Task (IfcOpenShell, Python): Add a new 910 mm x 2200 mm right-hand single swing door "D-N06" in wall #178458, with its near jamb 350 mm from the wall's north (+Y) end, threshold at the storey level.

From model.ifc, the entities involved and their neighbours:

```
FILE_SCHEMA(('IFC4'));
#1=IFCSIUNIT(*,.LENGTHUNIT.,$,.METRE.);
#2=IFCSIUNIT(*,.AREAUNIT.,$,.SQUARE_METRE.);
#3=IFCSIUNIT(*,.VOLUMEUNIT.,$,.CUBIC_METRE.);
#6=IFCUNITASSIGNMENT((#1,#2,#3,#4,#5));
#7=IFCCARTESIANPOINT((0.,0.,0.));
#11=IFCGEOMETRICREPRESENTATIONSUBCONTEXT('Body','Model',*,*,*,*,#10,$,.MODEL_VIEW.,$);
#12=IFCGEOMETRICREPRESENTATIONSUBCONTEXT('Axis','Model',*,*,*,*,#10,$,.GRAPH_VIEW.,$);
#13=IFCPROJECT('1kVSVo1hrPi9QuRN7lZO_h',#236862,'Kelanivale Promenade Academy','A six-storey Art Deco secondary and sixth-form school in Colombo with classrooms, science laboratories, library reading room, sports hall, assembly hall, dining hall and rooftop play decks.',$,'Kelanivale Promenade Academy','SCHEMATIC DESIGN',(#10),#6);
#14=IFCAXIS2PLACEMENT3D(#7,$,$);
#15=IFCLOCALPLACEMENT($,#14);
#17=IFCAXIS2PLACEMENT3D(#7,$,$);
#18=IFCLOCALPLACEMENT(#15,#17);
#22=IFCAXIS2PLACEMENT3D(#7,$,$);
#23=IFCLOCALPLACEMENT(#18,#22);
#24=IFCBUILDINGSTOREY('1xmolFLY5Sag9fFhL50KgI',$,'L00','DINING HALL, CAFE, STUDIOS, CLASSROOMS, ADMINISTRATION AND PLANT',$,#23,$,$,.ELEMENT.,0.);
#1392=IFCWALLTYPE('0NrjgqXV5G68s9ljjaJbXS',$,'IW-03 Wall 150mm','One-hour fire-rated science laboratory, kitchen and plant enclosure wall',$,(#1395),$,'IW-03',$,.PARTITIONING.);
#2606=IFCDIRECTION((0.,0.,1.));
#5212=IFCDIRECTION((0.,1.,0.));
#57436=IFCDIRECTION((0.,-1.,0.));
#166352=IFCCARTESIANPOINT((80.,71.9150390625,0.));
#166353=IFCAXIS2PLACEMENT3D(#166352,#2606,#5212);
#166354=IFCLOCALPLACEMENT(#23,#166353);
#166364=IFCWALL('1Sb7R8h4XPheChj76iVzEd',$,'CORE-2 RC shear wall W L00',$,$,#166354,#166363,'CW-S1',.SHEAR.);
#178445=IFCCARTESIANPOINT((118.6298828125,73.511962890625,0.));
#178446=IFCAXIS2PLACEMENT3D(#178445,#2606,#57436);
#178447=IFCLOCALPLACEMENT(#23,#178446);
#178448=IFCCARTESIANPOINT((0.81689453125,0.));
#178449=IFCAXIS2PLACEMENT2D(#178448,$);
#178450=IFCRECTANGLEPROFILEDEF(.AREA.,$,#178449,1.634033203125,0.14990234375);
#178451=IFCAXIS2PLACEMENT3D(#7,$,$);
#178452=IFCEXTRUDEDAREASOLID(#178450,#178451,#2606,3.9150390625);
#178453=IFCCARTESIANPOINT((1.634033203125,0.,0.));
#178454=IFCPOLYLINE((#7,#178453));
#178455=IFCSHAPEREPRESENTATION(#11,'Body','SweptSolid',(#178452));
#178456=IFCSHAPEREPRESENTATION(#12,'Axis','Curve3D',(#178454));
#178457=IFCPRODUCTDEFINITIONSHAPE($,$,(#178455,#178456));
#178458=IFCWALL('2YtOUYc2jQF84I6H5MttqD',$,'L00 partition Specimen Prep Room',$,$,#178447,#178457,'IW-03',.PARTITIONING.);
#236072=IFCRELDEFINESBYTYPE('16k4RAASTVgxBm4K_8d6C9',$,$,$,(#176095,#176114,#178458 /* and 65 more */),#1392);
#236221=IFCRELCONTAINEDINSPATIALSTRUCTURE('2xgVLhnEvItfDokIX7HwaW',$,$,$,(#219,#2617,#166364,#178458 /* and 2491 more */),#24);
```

```python
import numpy as np
import ifcopenshell
import ifcopenshell.api.feature
import ifcopenshell.api.geometry
import ifcopenshell.api.root
import ifcopenshell.api.spatial
import ifcopenshell.geom
import ifcopenshell.util.element
import ifcopenshell.util.placement
import ifcopenshell.util.representation
import ifcopenshell.util.shape
import ifcopenshell.util.unit

model = ifcopenshell.open("model.ifc")
unit_scale = ifcopenshell.util.unit.calculate_unit_scale(model)
settings = ifcopenshell.geom.settings()


def volume(element):
    """Net volume in cubic metres, openings subtracted."""
    shape = ifcopenshell.geom.create_shape(settings, element)
    return ifcopenshell.util.shape.get_volume(shape.geometry)


wall = model.by_guid("2YtOUYc2jQF84I6H5MttqD")
storey = ifcopenshell.util.element.get_container(wall, ifc_class="IfcBuildingStorey")
context = ifcopenshell.util.representation.get_context(model, "Model", "Body", "MODEL_VIEW")
before = volume(wall)

width, height, from_end, sill = 0.91, 2.2, 0.35, 0.0  # metres

# The wall runs along its own X axis, and the end named is its -X end.
wall_shape = ifcopenshell.geom.create_shape(settings, wall)
x, y, z = ifcopenshell.util.shape.get_vertices(wall_shape.geometry).T
start = x.min() + from_end
face, thickness = float(y.min()), float(y.max() - y.min())
wall_matrix = ifcopenshell.util.placement.get_local_placement(wall.ObjectPlacement)
level = ifcopenshell.util.placement.get_local_placement(storey.ObjectPlacement)[2, 3]


def in_wall(x, y):
    """Placement at x, y metres in the wall's axes, at sill height."""
    matrix = wall_matrix.copy()
    matrix[:, 3] = wall_matrix @ np.array([x / unit_scale, y / unit_scale, 0.0, 1.0])
    matrix[2, 3] = level + sill / unit_scale
    return matrix


# Opening: a box that overshoots both wall faces by 50 mm.
opening = ifcopenshell.api.root.create_entity(model, ifc_class="IfcOpeningElement", predefined_type="OPENING")
box = ifcopenshell.api.geometry.add_wall_representation(
    model, context=context, length=width, height=height, thickness=thickness + 0.1
)
ifcopenshell.api.geometry.assign_representation(model, product=opening, representation=box)
ifcopenshell.api.geometry.edit_object_placement(model, product=opening, matrix=in_wall(start, face - 0.05), is_si=False)
ifcopenshell.api.feature.add_feature(model, feature=opening, element=wall)

door = ifcopenshell.api.root.create_entity(model, ifc_class="IfcDoor", name="D-N06", predefined_type="DOOR")
door.OverallWidth, door.OverallHeight = width / unit_scale, height / unit_scale
door.OperationType = "SINGLE_SWING_RIGHT"
body = ifcopenshell.api.geometry.add_door_representation(
    model,
    context=context,
    overall_width=door.OverallWidth,
    overall_height=door.OverallHeight,
    operation_type="SINGLE_SWING_RIGHT",
    lining_properties={"LiningDepth": thickness / unit_scale, "ThresholdDepth": thickness / unit_scale},
)
ifcopenshell.api.geometry.assign_representation(model, product=door, representation=body)
ifcopenshell.api.spatial.assign_container(model, products=[door], relating_structure=storey)
ifcopenshell.api.feature.add_filling(model, opening=opening, element=door)

# The lining spans the wall, so the door starts at the wall face.
ifcopenshell.api.geometry.edit_object_placement(model, product=door, matrix=in_wall(start, face), is_si=False)

after = volume(wall)

print(f"wall volume {before:.3f} -> {after:.3f} m3")

model.write("model_v2.ifc")
```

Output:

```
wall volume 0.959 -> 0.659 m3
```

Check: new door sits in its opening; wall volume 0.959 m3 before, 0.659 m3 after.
